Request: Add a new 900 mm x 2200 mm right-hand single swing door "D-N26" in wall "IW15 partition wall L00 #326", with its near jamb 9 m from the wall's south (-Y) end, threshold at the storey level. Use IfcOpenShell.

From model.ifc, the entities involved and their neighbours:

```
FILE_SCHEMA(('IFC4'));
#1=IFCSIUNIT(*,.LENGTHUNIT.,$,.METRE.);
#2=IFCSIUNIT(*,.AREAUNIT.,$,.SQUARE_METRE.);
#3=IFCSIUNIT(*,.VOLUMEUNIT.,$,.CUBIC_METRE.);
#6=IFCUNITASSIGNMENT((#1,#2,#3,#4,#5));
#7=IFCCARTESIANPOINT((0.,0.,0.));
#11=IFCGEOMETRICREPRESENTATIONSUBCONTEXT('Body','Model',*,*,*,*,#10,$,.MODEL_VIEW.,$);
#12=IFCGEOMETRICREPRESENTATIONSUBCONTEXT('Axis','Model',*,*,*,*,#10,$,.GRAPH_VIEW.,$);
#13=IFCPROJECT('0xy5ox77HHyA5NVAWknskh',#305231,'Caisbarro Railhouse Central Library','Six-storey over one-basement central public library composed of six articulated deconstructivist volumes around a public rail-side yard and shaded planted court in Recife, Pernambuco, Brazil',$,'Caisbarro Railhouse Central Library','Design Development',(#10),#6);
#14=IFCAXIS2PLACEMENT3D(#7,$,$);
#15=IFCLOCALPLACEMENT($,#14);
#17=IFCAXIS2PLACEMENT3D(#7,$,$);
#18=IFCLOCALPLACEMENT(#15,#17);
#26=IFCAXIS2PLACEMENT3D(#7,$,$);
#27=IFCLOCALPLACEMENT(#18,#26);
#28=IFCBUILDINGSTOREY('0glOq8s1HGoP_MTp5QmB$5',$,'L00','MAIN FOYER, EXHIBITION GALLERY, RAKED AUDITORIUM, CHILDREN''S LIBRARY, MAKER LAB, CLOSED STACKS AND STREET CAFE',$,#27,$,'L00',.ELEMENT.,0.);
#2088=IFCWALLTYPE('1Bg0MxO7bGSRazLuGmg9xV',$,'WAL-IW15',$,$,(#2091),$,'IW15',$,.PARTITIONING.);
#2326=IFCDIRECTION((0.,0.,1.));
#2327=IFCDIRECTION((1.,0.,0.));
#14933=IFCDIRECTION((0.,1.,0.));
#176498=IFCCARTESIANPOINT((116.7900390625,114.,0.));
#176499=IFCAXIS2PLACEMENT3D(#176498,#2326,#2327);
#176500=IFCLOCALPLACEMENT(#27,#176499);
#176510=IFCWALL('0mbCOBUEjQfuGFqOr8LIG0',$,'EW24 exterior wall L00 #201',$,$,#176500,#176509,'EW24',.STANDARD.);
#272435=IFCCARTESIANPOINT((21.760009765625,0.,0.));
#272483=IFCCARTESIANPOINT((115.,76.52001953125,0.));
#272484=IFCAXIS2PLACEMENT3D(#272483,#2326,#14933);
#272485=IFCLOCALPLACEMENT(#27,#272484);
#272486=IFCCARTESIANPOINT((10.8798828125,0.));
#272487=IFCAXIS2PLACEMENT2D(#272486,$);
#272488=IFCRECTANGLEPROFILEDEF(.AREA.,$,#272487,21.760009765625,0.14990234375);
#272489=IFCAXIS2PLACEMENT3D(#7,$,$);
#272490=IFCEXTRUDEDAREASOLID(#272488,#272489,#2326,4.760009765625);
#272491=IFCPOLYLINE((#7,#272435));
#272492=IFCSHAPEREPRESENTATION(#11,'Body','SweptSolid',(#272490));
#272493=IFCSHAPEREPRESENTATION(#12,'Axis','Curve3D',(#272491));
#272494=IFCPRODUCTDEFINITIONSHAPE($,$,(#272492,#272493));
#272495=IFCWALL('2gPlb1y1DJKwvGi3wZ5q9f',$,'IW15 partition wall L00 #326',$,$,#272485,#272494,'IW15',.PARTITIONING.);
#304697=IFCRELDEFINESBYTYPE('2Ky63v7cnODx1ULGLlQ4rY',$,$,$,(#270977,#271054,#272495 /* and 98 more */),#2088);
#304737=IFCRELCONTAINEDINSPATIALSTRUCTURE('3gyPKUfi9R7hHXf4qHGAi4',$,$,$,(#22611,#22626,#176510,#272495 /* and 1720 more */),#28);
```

```python
import numpy as np
import ifcopenshell
import ifcopenshell.api.feature
import ifcopenshell.api.geometry
import ifcopenshell.api.root
import ifcopenshell.api.spatial
import ifcopenshell.geom
import ifcopenshell.util.element
import ifcopenshell.util.placement
import ifcopenshell.util.representation
import ifcopenshell.util.shape
import ifcopenshell.util.unit

model = ifcopenshell.open("model.ifc")
unit_scale = ifcopenshell.util.unit.calculate_unit_scale(model)
settings = ifcopenshell.geom.settings()


def volume(element):
    """Net volume in cubic metres, openings subtracted."""
    shape = ifcopenshell.geom.create_shape(settings, element)
    return ifcopenshell.util.shape.get_volume(shape.geometry)


wall = model.by_guid("2gPlb1y1DJKwvGi3wZ5q9f")
storey = ifcopenshell.util.element.get_container(wall, ifc_class="IfcBuildingStorey")
context = ifcopenshell.util.representation.get_context(model, "Model", "Body", "MODEL_VIEW")
before = volume(wall)

width, height, from_end, sill = 0.9, 2.2, 9, 0.0  # metres

# The wall runs along its own X axis, and the end named is its -X end.
wall_shape = ifcopenshell.geom.create_shape(settings, wall)
x, y, z = ifcopenshell.util.shape.get_vertices(wall_shape.geometry).T
start = x.min() + from_end
face, thickness = float(y.min()), float(y.max() - y.min())
wall_matrix = ifcopenshell.util.placement.get_local_placement(wall.ObjectPlacement)
level = ifcopenshell.util.placement.get_local_placement(storey.ObjectPlacement)[2, 3]


def in_wall(x, y):
    """Placement at x, y metres in the wall's axes, at sill height."""
    matrix = wall_matrix.copy()
    matrix[:, 3] = wall_matrix @ np.array([x / unit_scale, y / unit_scale, 0.0, 1.0])
    matrix[2, 3] = level + sill / unit_scale
    return matrix


# Opening: a box that overshoots both wall faces by 50 mm.
opening = ifcopenshell.api.root.create_entity(model, ifc_class="IfcOpeningElement", predefined_type="OPENING")
box = ifcopenshell.api.geometry.add_wall_representation(
    model, context=context, length=width, height=height, thickness=thickness + 0.1
)
ifcopenshell.api.geometry.assign_representation(model, product=opening, representation=box)
ifcopenshell.api.geometry.edit_object_placement(model, product=opening, matrix=in_wall(start, face - 0.05), is_si=False)
ifcopenshell.api.feature.add_feature(model, feature=opening, element=wall)

door = ifcopenshell.api.root.create_entity(model, ifc_class="IfcDoor", name="D-N26", predefined_type="DOOR")
door.OverallWidth, door.OverallHeight = width / unit_scale, height / unit_scale
door.OperationType = "SINGLE_SWING_RIGHT"
body = ifcopenshell.api.geometry.add_door_representation(
    model,
    context=context,
    overall_width=door.OverallWidth,
    overall_height=door.OverallHeight,
    operation_type="SINGLE_SWING_RIGHT",
    lining_properties={"LiningDepth": thickness / unit_scale, "ThresholdDepth": thickness / unit_scale},
)
ifcopenshell.api.geometry.assign_representation(model, product=door, representation=body)
ifcopenshell.api.spatial.assign_container(model, products=[door], relating_structure=storey)
ifcopenshell.api.feature.add_filling(model, opening=opening, element=door)

# The lining spans the wall, so the door starts at the wall face.
ifcopenshell.api.geometry.edit_object_placement(model, product=door, matrix=in_wall(start, face), is_si=False)

after = volume(wall)

print(f"wall volume {before:.3f} -> {after:.3f} m3")

model.write("model_v2.ifc")
```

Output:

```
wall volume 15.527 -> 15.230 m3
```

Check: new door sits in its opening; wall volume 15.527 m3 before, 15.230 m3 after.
